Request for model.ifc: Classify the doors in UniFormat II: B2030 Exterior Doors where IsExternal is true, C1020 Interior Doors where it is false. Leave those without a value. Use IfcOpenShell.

First a look at what the model holds.

```python
import ifcopenshell
import ifcopenshell.util.element

model = ifcopenshell.open("model.ifc")
print(model.schema)
print("classifications:", [c.Name for c in model.by_type("IfcClassification")])
values = [ifcopenshell.util.element.get_pset(e, "Pset_DoorCommon", "IsExternal") for e in model.by_type("IfcDoor")]
for value in (True, False, None):
    print("IsExternal", value, values.count(value))
```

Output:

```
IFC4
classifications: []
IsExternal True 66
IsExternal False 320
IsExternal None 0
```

```python
import ifcopenshell
import ifcopenshell.api.classification
import ifcopenshell.util.element

model = ifcopenshell.open("model.ifc")

system = ifcopenshell.api.classification.add_classification(model, classification="UniFormat II")

doors = model.by_type("IfcDoor")
external = {e: ifcopenshell.util.element.get_pset(e, "Pset_DoorCommon", "IsExternal") for e in doors}
for flag, code, name in ((True, "B2030", "Exterior Doors"), (False, "C1020", "Interior Doors")):
    products = [e for e in doors if external[e] is flag]
    ifcopenshell.api.classification.add_reference(
        model, products=products, classification=system, identification=code, name=name
    )
    print(code, len(products))

model.write("model_v2.ifc")
```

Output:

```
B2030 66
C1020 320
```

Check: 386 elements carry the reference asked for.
